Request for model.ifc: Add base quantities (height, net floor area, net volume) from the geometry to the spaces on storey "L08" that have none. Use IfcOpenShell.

First a look at what the model holds.

```python
import ifcopenshell
import ifcopenshell.util.element
import ifcopenshell.util.unit

model = ifcopenshell.open("model.ifc")
print(model.schema)
for unit_type in ("LENGTHUNIT", "AREAUNIT", "VOLUMEUNIT"):
    print(unit_type, ifcopenshell.util.unit.calculate_unit_scale(model, unit_type))
storey = next(s for s in model.by_type("IfcBuildingStorey") if s.Name == "L08")
spaces = [e for e in ifcopenshell.util.element.get_decomposition(storey) if e.is_a("IfcSpace")]
for e in sorted(spaces, key=lambda e: e.id()):
    print(e.id(), e.is_a(), e.Name, list(ifcopenshell.util.element.get_psets(e, qtos_only=True)), sep=" | ")
```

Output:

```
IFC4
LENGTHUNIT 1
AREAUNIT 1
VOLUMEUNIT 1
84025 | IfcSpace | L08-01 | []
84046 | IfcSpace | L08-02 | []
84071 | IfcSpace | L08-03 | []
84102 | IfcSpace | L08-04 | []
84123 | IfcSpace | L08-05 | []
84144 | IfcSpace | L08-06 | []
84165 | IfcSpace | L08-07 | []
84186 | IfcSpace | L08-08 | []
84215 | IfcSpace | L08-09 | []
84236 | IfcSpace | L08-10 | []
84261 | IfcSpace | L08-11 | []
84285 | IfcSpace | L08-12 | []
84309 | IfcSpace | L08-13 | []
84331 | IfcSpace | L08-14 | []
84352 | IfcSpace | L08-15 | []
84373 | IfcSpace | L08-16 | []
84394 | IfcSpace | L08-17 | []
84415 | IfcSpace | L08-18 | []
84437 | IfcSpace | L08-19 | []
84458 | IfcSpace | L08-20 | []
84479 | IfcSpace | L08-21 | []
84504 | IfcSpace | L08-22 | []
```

```python
import ifcopenshell
import ifcopenshell.api.pset
import ifcopenshell.geom
import ifcopenshell.util.element
import ifcopenshell.util.shape
import ifcopenshell.util.unit

model = ifcopenshell.open("model.ifc")
unit_scale = ifcopenshell.util.unit.calculate_unit_scale(model)
area_scale = ifcopenshell.util.unit.calculate_unit_scale(model, "AREAUNIT")
volume_scale = ifcopenshell.util.unit.calculate_unit_scale(model, "VOLUMEUNIT")
settings = ifcopenshell.geom.settings()

storey = next(s for s in model.by_type("IfcBuildingStorey") if s.Name == "L08")
spaces = [e for e in ifcopenshell.util.element.get_decomposition(storey) if e.is_a("IfcSpace")]

for e in sorted(spaces, key=lambda e: e.id()):
    if ifcopenshell.util.element.get_psets(e, qtos_only=True, should_inherit=False):
        continue
    # Geometry comes back in metres, in the element's own axes.
    shape = ifcopenshell.geom.create_shape(settings, e)
    values = {
        "Height": ifcopenshell.util.shape.get_z(shape.geometry) / unit_scale,
        "NetFloorArea": ifcopenshell.util.shape.get_footprint_area(shape.geometry) / area_scale,
        "NetVolume": ifcopenshell.util.shape.get_volume(shape.geometry) / volume_scale,
    }
    qto = ifcopenshell.api.pset.add_qto(model, product=e, name="Qto_SpaceBaseQuantities")
    ifcopenshell.api.pset.edit_qto(model, qto=qto, properties=values)
    print(e.id(), {k: round(v, 3) for k, v in values.items()})

model.write("model_v2.ifc")
```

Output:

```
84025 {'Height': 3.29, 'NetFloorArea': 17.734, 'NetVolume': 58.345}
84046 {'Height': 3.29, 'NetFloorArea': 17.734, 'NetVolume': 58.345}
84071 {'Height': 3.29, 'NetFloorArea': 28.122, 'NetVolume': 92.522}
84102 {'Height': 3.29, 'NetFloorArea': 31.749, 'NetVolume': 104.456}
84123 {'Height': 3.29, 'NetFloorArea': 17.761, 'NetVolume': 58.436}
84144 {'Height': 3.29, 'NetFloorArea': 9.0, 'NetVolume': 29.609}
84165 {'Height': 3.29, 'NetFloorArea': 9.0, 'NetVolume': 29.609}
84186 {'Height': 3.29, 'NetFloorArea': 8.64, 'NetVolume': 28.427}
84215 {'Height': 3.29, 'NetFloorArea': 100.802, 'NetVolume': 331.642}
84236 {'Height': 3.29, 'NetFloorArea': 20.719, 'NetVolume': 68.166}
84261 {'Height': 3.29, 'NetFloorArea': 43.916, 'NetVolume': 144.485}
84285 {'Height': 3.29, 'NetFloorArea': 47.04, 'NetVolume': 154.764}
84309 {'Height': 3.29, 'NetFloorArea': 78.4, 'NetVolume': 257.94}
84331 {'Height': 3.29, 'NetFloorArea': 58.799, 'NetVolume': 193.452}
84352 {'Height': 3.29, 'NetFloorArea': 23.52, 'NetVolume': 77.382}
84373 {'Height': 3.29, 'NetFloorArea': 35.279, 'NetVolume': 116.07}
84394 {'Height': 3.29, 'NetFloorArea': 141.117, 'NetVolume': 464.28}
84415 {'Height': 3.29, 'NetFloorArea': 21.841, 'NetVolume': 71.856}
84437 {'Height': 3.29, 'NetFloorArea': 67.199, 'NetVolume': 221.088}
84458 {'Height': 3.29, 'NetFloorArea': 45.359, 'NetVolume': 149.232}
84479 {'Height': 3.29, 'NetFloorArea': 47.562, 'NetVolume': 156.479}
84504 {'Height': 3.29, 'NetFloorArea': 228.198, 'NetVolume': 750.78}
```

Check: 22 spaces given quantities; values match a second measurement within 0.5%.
